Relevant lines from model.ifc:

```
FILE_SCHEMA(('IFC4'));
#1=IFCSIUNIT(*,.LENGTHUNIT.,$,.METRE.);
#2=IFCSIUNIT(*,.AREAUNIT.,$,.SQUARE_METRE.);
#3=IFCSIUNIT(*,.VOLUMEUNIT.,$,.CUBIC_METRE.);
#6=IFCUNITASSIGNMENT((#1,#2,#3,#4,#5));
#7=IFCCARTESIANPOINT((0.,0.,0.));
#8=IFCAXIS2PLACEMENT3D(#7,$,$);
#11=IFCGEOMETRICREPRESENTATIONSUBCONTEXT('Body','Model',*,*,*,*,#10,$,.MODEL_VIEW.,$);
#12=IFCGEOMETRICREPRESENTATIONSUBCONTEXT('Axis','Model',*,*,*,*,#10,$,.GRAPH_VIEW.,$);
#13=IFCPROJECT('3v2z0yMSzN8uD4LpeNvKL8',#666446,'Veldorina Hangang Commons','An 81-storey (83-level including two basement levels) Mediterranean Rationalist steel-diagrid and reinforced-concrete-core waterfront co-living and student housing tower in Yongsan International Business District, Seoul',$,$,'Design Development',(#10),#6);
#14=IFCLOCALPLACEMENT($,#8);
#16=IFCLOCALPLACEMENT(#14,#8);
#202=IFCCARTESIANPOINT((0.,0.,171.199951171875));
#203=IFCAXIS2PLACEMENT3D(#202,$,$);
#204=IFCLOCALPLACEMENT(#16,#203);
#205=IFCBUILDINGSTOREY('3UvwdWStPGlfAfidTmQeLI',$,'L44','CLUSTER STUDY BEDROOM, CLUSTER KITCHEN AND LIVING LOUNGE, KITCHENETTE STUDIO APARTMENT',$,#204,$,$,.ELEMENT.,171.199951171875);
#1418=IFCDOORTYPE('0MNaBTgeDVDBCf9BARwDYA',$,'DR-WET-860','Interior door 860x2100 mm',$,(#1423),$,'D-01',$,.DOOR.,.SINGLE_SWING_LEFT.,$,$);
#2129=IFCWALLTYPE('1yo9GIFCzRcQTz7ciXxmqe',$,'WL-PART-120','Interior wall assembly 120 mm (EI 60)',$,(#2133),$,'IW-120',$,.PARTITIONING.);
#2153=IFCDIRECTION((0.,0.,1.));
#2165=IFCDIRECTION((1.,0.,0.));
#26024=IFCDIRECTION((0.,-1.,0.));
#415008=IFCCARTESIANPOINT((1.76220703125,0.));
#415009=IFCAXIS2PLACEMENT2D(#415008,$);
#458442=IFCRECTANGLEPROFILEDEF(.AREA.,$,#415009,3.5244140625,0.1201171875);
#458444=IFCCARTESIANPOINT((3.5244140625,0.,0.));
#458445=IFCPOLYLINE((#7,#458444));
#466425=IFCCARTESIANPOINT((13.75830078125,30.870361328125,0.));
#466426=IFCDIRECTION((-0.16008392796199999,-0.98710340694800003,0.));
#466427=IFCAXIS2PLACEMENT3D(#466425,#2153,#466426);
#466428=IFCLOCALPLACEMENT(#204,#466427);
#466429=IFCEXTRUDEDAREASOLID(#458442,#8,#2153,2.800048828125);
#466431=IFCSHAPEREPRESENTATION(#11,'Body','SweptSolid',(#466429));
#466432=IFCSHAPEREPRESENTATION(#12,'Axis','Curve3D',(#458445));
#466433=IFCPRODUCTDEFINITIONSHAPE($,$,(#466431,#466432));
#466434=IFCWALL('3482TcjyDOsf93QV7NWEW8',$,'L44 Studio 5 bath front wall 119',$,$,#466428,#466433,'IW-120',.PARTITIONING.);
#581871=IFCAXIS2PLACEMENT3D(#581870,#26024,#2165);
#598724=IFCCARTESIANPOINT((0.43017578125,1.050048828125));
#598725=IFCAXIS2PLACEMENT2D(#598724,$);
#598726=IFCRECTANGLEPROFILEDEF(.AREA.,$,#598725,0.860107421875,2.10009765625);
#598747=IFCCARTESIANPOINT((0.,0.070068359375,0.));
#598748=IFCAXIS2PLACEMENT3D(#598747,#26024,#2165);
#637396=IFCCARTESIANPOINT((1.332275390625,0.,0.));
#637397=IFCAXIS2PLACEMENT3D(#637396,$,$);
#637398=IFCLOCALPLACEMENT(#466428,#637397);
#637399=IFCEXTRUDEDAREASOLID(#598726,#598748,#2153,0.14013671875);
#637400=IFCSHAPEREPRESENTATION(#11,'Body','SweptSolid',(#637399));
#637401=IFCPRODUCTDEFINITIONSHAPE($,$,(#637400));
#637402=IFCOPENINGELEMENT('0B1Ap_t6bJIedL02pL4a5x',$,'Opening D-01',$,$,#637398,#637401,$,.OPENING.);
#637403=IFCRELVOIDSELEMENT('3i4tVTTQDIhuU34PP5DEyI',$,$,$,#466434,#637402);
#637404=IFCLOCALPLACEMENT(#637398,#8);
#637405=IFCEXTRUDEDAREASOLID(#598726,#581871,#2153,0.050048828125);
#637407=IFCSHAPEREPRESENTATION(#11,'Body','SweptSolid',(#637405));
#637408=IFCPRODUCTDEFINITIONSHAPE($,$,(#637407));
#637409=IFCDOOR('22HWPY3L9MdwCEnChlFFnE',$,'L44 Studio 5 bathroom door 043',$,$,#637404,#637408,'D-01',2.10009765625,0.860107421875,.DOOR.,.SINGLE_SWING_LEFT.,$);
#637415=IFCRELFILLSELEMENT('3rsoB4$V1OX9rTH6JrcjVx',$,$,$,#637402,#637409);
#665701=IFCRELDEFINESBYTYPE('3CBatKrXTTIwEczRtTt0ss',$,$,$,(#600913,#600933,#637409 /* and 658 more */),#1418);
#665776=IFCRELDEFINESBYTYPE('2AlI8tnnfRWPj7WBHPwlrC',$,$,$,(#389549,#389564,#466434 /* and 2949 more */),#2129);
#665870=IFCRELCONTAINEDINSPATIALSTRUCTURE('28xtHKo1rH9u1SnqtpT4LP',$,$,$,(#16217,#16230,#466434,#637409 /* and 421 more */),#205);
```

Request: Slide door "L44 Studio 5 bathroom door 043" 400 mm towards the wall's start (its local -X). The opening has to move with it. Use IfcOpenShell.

```python
import ifcopenshell
import ifcopenshell.api.geometry
import ifcopenshell.util.placement
import ifcopenshell.util.unit

model = ifcopenshell.open("model.ifc")
unit_scale = ifcopenshell.util.unit.calculate_unit_scale(model)

door = model.by_guid("22HWPY3L9MdwCEnChlFFnE")
opening = door.FillsVoids[0].RelatingOpeningElement
wall = opening.VoidsElements[0].RelatingBuildingElement

wall_matrix = ifcopenshell.util.placement.get_local_placement(wall.ObjectPlacement)
shift = wall_matrix[:3, 0] * -0.4 / unit_scale
before = ifcopenshell.util.placement.get_local_placement(door.ObjectPlacement)[:3, 3].copy()

# The door is placed relative to its opening, so it follows when the opening moves.
matrix = ifcopenshell.util.placement.get_local_placement(opening.ObjectPlacement)
matrix[:3, 3] += shift
ifcopenshell.api.geometry.edit_object_placement(
    model, product=opening, matrix=matrix, is_si=False, should_transform_children=True
)

after = ifcopenshell.util.placement.get_local_placement(door.ObjectPlacement)[:3, 3]
print("door moved by", (after - before).round(3) + 0.0)

model.write("model_rev.ifc")
```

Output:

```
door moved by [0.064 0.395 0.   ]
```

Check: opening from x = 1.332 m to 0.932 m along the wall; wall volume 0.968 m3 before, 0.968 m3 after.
